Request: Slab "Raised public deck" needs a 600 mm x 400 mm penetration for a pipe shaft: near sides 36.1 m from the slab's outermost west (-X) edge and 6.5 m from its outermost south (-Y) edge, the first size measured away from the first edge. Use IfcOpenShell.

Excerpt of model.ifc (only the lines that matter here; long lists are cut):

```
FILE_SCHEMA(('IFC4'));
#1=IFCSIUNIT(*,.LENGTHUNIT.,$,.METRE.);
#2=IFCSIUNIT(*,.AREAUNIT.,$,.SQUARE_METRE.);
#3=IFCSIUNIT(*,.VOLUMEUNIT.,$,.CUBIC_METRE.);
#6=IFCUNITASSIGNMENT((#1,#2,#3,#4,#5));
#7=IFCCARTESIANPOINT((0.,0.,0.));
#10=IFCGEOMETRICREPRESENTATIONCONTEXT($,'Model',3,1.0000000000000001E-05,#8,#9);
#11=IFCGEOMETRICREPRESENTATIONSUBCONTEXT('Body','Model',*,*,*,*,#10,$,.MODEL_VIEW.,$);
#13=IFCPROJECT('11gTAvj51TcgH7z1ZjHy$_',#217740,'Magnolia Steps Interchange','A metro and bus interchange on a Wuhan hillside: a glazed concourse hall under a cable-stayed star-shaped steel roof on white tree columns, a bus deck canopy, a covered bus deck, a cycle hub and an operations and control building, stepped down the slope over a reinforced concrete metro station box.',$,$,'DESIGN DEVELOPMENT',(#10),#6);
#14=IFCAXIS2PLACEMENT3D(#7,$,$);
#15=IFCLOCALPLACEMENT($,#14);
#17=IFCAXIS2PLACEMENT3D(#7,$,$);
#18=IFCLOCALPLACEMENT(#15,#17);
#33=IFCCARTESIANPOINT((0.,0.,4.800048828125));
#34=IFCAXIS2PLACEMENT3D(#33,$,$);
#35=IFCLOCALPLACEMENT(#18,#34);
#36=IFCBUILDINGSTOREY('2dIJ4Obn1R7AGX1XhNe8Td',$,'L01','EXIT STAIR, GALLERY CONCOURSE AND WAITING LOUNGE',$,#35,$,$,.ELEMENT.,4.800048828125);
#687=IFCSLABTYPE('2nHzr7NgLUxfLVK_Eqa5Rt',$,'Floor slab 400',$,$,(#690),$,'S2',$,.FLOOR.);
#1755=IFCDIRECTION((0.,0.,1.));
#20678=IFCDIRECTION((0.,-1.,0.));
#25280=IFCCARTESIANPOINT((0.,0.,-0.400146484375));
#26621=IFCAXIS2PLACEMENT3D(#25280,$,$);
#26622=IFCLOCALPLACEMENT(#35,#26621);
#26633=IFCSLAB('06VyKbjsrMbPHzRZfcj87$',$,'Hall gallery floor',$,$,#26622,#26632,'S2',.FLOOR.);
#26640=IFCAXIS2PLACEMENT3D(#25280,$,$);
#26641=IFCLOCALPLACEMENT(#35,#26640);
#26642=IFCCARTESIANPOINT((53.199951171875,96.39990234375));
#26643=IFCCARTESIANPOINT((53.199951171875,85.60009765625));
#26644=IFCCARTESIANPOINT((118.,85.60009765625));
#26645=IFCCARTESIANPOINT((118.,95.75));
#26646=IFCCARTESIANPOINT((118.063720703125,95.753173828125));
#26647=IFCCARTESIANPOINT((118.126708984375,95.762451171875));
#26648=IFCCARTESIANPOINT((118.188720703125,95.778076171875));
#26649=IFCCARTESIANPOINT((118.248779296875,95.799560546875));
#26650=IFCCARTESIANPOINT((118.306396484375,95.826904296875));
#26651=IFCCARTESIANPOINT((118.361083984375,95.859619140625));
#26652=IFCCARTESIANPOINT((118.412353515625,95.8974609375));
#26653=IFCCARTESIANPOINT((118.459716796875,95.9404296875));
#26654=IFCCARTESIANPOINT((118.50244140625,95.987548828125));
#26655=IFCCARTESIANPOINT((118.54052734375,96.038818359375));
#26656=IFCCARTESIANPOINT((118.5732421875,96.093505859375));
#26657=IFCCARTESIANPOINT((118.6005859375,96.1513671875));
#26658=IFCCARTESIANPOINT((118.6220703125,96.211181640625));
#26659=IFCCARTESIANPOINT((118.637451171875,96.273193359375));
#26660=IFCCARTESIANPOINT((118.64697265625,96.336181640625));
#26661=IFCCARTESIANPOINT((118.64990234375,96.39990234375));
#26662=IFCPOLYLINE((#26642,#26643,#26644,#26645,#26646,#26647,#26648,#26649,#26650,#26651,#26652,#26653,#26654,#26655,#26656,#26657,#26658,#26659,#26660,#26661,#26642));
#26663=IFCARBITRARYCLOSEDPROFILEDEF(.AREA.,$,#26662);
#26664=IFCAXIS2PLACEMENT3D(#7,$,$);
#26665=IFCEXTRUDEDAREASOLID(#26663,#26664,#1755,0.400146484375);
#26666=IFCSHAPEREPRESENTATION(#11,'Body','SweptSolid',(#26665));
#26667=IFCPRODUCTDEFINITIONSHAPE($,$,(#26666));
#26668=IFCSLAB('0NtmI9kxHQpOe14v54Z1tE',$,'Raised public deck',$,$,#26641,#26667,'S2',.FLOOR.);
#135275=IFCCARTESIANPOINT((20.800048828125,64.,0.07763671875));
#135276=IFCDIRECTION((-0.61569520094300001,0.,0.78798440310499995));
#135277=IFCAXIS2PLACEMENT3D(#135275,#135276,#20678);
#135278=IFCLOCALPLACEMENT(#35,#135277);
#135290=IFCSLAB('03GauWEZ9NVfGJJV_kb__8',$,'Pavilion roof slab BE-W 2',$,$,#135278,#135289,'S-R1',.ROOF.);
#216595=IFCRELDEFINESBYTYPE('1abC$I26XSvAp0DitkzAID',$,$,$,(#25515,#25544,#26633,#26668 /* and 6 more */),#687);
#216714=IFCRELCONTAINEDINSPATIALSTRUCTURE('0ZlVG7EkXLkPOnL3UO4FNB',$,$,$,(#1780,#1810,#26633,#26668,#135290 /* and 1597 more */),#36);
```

```python
import numpy as np
import ifcopenshell
import ifcopenshell.api.feature
import ifcopenshell.api.geometry
import ifcopenshell.api.root
import ifcopenshell.geom
import ifcopenshell.util.placement
import ifcopenshell.util.representation
import ifcopenshell.util.shape
import ifcopenshell.util.unit

model = ifcopenshell.open("model.ifc")
unit_scale = ifcopenshell.util.unit.calculate_unit_scale(model)
settings = ifcopenshell.geom.settings()


def volume(element):
    """Net volume in cubic metres, openings subtracted."""
    shape = ifcopenshell.geom.create_shape(settings, element)
    return ifcopenshell.util.shape.get_volume(shape.geometry)


slab = model.by_guid("0NtmI9kxHQpOe14v54Z1tE")
before = volume(slab)

# Extent in the slab's own axes, in metres. The edges named are its -X and -Y sides.
slab_shape = ifcopenshell.geom.create_shape(settings, slab)
vertices = ifcopenshell.util.shape.get_vertices(slab_shape.geometry)
x_min, y_min, bottom = vertices.min(axis=0)
top = vertices[:, 2].max()

opening = ifcopenshell.api.root.create_entity(model, ifc_class="IfcOpeningElement", name="Pipe shaft opening", predefined_type="OPENING")
context = ifcopenshell.util.representation.get_context(model, "Model", "Body", "MODEL_VIEW")
width, depth = 0.6, 0.4
outline = [(0.0, 0.0), (width, 0.0), (width, depth), (0.0, depth), (0.0, 0.0)]
# Overshoot both faces by 50 mm so the cut is clean.
shape = ifcopenshell.api.geometry.add_slab_representation(
    model, context=context, depth=top - bottom + 0.1, polyline=outline
)
ifcopenshell.api.geometry.assign_representation(model, product=opening, representation=shape)

matrix = ifcopenshell.util.placement.get_local_placement(slab.ObjectPlacement)
matrix[:, 3] = matrix @ np.append(np.array([x_min + 36.1, y_min + 6.5, bottom - 0.05]) / unit_scale, 1.0)
ifcopenshell.api.geometry.edit_object_placement(model, product=opening, matrix=matrix, is_si=False)
ifcopenshell.api.feature.add_feature(model, feature=opening, element=slab)

after = volume(slab)

print(f"slab volume {before:.3f} -> {after:.3f} m3")

model.write("model_updated.ifc")
```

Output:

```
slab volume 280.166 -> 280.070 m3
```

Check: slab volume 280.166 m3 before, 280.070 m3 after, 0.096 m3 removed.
